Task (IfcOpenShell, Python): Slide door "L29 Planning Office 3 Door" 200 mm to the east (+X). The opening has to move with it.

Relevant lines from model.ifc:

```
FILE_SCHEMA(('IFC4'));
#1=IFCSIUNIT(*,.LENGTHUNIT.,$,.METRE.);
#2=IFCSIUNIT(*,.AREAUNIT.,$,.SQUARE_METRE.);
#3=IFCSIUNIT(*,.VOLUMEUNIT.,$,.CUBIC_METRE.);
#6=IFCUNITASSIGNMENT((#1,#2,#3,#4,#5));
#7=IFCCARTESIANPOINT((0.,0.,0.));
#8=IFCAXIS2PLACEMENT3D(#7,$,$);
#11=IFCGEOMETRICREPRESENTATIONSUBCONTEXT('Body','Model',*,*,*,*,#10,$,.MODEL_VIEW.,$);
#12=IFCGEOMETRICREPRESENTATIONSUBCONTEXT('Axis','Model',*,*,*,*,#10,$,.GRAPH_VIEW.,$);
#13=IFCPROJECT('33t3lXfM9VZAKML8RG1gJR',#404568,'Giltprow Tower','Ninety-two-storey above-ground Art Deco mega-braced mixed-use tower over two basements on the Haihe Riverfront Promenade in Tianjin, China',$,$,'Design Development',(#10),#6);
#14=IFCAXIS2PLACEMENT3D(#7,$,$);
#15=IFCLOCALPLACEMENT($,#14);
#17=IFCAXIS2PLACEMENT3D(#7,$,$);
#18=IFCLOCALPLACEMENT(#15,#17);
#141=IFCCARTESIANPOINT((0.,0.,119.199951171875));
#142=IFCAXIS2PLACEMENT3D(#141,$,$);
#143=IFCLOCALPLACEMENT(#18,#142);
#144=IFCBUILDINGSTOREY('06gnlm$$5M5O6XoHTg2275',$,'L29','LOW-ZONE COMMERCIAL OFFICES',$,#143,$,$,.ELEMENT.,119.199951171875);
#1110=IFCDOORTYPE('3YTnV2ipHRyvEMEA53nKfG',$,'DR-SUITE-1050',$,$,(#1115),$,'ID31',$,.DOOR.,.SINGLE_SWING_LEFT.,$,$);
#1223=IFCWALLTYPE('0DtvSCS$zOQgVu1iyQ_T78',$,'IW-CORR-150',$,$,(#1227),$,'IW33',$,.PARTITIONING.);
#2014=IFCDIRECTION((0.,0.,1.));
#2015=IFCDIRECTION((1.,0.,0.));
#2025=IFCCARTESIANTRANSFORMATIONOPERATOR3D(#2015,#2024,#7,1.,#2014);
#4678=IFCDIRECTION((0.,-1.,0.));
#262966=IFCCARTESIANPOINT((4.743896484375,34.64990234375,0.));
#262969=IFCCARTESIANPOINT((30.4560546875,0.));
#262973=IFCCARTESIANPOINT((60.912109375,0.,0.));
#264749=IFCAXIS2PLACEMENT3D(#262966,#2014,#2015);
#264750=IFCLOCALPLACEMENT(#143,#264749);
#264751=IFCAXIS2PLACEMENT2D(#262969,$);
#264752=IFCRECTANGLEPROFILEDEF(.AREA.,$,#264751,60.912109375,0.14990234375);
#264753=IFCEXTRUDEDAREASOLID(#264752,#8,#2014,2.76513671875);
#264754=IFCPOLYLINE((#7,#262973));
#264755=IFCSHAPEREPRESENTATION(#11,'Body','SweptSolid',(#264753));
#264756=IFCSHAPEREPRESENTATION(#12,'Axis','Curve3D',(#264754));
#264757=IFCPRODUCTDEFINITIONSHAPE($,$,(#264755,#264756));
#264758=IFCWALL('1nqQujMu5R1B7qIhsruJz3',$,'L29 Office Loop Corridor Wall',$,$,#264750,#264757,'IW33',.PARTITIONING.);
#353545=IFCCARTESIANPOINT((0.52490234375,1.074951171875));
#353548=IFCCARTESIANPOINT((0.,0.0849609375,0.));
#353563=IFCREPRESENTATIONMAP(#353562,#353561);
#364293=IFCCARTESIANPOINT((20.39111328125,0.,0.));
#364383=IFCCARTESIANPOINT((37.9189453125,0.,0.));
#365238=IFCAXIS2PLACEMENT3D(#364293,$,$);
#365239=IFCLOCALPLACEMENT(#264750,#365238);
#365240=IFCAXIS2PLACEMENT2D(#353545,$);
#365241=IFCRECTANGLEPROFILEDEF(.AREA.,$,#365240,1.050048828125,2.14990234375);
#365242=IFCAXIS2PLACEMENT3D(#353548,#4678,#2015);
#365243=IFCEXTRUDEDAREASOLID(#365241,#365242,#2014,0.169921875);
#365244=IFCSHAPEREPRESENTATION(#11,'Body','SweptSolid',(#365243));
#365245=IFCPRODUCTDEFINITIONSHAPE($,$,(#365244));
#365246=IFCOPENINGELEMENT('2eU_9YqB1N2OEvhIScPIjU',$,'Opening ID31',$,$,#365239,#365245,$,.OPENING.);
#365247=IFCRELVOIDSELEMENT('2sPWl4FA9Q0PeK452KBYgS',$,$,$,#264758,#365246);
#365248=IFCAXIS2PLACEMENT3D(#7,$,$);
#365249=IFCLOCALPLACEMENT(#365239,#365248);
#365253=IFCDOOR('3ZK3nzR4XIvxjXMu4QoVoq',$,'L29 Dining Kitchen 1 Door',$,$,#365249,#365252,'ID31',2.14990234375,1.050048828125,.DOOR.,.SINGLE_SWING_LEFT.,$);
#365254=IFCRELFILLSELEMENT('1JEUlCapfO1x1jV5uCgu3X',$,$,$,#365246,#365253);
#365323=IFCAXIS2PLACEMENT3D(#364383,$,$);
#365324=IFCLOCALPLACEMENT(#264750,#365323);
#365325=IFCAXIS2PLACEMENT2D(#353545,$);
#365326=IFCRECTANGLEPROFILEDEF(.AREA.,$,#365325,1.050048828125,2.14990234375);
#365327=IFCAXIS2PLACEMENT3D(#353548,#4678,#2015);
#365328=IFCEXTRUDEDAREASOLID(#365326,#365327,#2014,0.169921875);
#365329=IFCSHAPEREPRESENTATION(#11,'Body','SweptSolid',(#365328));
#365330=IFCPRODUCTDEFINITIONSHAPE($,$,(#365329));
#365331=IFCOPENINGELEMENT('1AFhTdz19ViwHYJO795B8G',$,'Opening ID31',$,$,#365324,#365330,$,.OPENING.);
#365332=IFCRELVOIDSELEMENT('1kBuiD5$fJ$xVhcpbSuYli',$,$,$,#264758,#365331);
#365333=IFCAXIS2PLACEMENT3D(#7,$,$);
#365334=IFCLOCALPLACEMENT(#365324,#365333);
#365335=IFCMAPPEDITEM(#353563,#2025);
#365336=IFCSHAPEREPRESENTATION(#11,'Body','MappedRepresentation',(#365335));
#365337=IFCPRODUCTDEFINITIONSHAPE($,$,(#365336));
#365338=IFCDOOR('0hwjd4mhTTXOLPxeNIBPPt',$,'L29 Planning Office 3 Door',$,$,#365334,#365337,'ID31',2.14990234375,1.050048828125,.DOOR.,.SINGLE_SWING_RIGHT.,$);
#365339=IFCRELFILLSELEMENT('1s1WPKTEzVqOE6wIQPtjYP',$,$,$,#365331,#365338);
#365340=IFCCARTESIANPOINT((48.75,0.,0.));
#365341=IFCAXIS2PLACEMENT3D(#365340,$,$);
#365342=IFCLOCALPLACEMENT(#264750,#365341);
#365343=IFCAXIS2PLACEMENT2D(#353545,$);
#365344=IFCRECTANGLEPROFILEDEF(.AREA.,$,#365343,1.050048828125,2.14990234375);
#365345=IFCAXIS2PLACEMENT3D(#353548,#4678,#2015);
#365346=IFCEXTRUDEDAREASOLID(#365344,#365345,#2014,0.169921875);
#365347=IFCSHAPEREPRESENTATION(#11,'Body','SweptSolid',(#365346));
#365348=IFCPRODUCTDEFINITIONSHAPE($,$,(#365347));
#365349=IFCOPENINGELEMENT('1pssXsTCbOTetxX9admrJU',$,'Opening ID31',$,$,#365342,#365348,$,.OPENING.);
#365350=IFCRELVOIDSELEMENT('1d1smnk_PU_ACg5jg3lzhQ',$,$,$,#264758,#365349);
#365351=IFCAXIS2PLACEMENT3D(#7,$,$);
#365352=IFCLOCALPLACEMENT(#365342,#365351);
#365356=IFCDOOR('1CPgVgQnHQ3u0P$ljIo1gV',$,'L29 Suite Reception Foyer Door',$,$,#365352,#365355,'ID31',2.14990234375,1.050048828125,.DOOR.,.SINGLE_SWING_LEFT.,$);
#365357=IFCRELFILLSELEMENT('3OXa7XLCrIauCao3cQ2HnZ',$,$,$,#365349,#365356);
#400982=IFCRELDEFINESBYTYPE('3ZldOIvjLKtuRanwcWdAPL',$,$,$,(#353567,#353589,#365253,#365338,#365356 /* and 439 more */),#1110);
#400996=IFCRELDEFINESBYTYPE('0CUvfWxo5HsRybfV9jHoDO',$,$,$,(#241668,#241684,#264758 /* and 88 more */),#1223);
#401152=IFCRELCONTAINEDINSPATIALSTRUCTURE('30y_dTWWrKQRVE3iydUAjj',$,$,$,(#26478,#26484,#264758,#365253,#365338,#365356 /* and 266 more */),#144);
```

```python
import ifcopenshell
import ifcopenshell.api.geometry
import ifcopenshell.util.placement

model = ifcopenshell.open("model.ifc")

door = model.by_guid("0hwjd4mhTTXOLPxeNIBPPt")
opening = door.FillsVoids[0].RelatingOpeningElement
wall = opening.VoidsElements[0].RelatingBuildingElement

wall_matrix = ifcopenshell.util.placement.get_local_placement(wall.ObjectPlacement)
shift = wall_matrix[:3, 0] * 0.2
before = ifcopenshell.util.placement.get_local_placement(door.ObjectPlacement)[:3, 3].copy()

# The door is placed relative to its opening, so it follows when the opening moves.
matrix = ifcopenshell.util.placement.get_local_placement(opening.ObjectPlacement)
matrix[:3, 3] += shift
ifcopenshell.api.geometry.edit_object_placement(
    model, product=opening, matrix=matrix, is_si=False, should_transform_children=True
)

after = ifcopenshell.util.placement.get_local_placement(door.ObjectPlacement)[:3, 3]
print("door moved by", (after - before).round(3) + 0.0)

model.write("model_rev.ifc")
```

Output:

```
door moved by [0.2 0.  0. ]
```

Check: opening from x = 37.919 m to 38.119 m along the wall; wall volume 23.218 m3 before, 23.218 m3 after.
